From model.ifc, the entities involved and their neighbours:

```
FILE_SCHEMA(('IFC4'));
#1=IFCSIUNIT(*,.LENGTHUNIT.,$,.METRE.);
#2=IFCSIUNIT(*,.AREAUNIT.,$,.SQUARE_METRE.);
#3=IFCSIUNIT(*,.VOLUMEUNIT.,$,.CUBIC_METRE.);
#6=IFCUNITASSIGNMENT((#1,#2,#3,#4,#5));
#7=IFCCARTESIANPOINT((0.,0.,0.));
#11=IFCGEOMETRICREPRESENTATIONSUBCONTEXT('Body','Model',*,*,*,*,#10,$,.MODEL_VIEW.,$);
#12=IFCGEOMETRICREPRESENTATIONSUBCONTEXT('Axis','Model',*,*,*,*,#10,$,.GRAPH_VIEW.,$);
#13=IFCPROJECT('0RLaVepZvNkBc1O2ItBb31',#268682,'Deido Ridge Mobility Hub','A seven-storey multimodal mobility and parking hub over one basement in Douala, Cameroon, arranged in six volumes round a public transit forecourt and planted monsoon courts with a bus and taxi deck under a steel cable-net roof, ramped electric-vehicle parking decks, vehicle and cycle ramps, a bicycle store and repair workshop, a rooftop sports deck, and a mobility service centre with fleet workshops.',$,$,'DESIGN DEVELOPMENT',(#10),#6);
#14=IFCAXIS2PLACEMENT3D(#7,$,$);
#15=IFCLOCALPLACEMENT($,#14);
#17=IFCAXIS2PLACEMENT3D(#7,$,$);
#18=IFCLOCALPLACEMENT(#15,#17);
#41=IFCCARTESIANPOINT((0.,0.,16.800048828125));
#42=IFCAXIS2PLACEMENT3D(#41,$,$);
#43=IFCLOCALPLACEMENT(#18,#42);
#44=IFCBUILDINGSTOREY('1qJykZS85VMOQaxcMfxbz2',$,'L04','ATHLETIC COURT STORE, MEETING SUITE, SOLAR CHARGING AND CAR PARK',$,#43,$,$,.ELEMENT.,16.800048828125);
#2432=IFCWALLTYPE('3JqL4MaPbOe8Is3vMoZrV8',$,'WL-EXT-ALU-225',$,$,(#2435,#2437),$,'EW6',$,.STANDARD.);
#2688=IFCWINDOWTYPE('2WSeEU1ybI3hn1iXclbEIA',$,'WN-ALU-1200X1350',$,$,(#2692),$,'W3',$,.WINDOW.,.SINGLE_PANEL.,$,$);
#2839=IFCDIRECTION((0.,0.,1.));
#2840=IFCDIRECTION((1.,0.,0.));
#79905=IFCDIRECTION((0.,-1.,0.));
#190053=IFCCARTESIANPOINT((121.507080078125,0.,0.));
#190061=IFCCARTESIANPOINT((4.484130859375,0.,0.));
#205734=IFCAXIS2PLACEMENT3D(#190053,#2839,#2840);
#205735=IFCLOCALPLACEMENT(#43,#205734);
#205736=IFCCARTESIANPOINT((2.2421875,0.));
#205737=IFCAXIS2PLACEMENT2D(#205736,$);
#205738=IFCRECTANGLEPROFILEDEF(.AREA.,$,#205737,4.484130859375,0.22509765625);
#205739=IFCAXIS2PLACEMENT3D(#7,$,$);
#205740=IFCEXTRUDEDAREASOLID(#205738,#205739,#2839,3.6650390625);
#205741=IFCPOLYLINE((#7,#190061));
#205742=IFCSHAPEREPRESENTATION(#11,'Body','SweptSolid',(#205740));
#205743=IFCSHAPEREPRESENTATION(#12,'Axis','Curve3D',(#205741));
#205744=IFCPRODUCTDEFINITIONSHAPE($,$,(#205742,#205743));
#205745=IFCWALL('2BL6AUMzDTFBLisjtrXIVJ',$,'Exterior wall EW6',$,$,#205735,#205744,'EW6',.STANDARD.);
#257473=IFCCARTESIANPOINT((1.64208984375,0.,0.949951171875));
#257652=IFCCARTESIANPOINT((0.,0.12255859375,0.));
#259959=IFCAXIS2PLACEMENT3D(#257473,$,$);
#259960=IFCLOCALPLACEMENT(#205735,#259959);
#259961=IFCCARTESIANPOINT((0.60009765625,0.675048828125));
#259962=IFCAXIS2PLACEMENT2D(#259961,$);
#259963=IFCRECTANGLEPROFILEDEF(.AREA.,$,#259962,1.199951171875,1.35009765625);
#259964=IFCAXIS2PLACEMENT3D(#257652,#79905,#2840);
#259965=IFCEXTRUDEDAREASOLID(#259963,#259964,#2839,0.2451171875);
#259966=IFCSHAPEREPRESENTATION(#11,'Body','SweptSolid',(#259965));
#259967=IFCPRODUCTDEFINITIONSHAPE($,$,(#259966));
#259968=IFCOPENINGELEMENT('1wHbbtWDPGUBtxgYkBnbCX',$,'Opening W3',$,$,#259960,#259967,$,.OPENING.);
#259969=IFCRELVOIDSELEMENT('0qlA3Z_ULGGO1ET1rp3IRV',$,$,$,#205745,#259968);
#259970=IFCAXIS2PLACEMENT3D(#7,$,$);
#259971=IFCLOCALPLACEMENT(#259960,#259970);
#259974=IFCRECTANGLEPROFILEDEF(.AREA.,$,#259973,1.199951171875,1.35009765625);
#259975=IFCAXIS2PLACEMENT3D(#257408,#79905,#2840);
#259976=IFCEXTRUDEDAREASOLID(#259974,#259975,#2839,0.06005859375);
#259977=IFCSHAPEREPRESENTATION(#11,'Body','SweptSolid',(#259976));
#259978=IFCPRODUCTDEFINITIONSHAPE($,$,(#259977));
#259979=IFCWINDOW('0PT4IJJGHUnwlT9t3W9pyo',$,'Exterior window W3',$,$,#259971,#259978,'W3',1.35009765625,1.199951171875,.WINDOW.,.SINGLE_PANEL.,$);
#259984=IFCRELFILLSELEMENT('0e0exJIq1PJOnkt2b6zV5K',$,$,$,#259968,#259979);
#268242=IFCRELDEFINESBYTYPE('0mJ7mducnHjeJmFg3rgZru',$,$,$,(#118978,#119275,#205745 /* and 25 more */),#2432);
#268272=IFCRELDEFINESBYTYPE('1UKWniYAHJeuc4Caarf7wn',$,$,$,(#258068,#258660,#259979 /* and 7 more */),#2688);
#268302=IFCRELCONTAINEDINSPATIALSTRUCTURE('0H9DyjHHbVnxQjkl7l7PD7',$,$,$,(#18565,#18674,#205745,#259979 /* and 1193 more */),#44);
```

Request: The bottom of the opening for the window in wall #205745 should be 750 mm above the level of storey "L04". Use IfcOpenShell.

```python
import numpy as np
import ifcopenshell
import ifcopenshell.api.geometry
import ifcopenshell.geom
import ifcopenshell.util.element
import ifcopenshell.util.placement
import ifcopenshell.util.shape
import ifcopenshell.util.unit

model = ifcopenshell.open("model.ifc")
unit_scale = ifcopenshell.util.unit.calculate_unit_scale(model)

window = model.by_guid("0PT4IJJGHUnwlT9t3W9pyo")
opening = window.FillsVoids[0].RelatingOpeningElement
storey = ifcopenshell.util.element.get_container(window, ifc_class="IfcBuildingStorey")
level = ifcopenshell.util.placement.get_local_placement(storey.ObjectPlacement)[2, 3]

# The opening's origin need not be at the sill, so measure its lowest point.
shape = ifcopenshell.geom.create_shape(ifcopenshell.geom.settings(), opening)
bottom = ifcopenshell.util.shape.get_shape_bottom_elevation(shape, shape.geometry) / unit_scale
dz = level + 0.75 / unit_scale - bottom

shift = np.array([0.0, 0.0, dz])
# The window is placed relative to its opening, so it follows when the opening moves.
matrix = ifcopenshell.util.placement.get_local_placement(opening.ObjectPlacement)
matrix[:3, 3] += shift
ifcopenshell.api.geometry.edit_object_placement(
    model, product=opening, matrix=matrix, is_si=False, should_transform_children=True
)

print(f"moved by {dz * unit_scale:+.3f} m")

model.write("model_edited.ifc")
```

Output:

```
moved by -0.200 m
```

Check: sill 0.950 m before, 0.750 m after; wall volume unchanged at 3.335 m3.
